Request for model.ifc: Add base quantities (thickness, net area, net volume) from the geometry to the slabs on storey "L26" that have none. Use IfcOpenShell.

First a look at what the model holds.

```python
import ifcopenshell
import ifcopenshell.util.element
import ifcopenshell.util.unit

model = ifcopenshell.open("model.ifc")
print(model.schema)
for unit_type in ("LENGTHUNIT", "AREAUNIT", "VOLUMEUNIT"):
    print(unit_type, ifcopenshell.util.unit.calculate_unit_scale(model, unit_type))
storey = next(s for s in model.by_type("IfcBuildingStorey") if s.Name == "L26")
slabs = [e for e in ifcopenshell.util.element.get_decomposition(storey) if e.is_a("IfcSlab")]
for e in sorted(slabs, key=lambda e: e.id()):
    print(e.id(), e.is_a(), e.Name, list(ifcopenshell.util.element.get_psets(e, qtos_only=True)), sep=" | ")
```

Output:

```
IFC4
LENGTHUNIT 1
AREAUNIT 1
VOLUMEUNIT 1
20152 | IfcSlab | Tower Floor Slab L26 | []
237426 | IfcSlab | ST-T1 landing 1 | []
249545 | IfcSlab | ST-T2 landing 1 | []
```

```python
import ifcopenshell
import ifcopenshell.api.pset
import ifcopenshell.geom
import ifcopenshell.util.element
import ifcopenshell.util.shape
import ifcopenshell.util.unit

model = ifcopenshell.open("model.ifc")
unit_scale = ifcopenshell.util.unit.calculate_unit_scale(model)
area_scale = ifcopenshell.util.unit.calculate_unit_scale(model, "AREAUNIT")
volume_scale = ifcopenshell.util.unit.calculate_unit_scale(model, "VOLUMEUNIT")
settings = ifcopenshell.geom.settings()

storey = next(s for s in model.by_type("IfcBuildingStorey") if s.Name == "L26")
slabs = [e for e in ifcopenshell.util.element.get_decomposition(storey) if e.is_a("IfcSlab")]

for e in sorted(slabs, key=lambda e: e.id()):
    if ifcopenshell.util.element.get_psets(e, qtos_only=True, should_inherit=False):
        continue
    # Geometry comes back in metres, in the element's own axes.
    shape = ifcopenshell.geom.create_shape(settings, e)
    values = {
        "Width": ifcopenshell.util.shape.get_z(shape.geometry) / unit_scale,
        "NetArea": ifcopenshell.util.shape.get_footprint_area(shape.geometry) / area_scale,
        "NetVolume": ifcopenshell.util.shape.get_volume(shape.geometry) / volume_scale,
    }
    qto = ifcopenshell.api.pset.add_qto(model, product=e, name="Qto_SlabBaseQuantities")
    ifcopenshell.api.pset.edit_qto(model, qto=qto, properties=values)
    print(e.id(), {k: round(v, 3) for k, v in values.items()})

model.write("model_v2.ifc")
```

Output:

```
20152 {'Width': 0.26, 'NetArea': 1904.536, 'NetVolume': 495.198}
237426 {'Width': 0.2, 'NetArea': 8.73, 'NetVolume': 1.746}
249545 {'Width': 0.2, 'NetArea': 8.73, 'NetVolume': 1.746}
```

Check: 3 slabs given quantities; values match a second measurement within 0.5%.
